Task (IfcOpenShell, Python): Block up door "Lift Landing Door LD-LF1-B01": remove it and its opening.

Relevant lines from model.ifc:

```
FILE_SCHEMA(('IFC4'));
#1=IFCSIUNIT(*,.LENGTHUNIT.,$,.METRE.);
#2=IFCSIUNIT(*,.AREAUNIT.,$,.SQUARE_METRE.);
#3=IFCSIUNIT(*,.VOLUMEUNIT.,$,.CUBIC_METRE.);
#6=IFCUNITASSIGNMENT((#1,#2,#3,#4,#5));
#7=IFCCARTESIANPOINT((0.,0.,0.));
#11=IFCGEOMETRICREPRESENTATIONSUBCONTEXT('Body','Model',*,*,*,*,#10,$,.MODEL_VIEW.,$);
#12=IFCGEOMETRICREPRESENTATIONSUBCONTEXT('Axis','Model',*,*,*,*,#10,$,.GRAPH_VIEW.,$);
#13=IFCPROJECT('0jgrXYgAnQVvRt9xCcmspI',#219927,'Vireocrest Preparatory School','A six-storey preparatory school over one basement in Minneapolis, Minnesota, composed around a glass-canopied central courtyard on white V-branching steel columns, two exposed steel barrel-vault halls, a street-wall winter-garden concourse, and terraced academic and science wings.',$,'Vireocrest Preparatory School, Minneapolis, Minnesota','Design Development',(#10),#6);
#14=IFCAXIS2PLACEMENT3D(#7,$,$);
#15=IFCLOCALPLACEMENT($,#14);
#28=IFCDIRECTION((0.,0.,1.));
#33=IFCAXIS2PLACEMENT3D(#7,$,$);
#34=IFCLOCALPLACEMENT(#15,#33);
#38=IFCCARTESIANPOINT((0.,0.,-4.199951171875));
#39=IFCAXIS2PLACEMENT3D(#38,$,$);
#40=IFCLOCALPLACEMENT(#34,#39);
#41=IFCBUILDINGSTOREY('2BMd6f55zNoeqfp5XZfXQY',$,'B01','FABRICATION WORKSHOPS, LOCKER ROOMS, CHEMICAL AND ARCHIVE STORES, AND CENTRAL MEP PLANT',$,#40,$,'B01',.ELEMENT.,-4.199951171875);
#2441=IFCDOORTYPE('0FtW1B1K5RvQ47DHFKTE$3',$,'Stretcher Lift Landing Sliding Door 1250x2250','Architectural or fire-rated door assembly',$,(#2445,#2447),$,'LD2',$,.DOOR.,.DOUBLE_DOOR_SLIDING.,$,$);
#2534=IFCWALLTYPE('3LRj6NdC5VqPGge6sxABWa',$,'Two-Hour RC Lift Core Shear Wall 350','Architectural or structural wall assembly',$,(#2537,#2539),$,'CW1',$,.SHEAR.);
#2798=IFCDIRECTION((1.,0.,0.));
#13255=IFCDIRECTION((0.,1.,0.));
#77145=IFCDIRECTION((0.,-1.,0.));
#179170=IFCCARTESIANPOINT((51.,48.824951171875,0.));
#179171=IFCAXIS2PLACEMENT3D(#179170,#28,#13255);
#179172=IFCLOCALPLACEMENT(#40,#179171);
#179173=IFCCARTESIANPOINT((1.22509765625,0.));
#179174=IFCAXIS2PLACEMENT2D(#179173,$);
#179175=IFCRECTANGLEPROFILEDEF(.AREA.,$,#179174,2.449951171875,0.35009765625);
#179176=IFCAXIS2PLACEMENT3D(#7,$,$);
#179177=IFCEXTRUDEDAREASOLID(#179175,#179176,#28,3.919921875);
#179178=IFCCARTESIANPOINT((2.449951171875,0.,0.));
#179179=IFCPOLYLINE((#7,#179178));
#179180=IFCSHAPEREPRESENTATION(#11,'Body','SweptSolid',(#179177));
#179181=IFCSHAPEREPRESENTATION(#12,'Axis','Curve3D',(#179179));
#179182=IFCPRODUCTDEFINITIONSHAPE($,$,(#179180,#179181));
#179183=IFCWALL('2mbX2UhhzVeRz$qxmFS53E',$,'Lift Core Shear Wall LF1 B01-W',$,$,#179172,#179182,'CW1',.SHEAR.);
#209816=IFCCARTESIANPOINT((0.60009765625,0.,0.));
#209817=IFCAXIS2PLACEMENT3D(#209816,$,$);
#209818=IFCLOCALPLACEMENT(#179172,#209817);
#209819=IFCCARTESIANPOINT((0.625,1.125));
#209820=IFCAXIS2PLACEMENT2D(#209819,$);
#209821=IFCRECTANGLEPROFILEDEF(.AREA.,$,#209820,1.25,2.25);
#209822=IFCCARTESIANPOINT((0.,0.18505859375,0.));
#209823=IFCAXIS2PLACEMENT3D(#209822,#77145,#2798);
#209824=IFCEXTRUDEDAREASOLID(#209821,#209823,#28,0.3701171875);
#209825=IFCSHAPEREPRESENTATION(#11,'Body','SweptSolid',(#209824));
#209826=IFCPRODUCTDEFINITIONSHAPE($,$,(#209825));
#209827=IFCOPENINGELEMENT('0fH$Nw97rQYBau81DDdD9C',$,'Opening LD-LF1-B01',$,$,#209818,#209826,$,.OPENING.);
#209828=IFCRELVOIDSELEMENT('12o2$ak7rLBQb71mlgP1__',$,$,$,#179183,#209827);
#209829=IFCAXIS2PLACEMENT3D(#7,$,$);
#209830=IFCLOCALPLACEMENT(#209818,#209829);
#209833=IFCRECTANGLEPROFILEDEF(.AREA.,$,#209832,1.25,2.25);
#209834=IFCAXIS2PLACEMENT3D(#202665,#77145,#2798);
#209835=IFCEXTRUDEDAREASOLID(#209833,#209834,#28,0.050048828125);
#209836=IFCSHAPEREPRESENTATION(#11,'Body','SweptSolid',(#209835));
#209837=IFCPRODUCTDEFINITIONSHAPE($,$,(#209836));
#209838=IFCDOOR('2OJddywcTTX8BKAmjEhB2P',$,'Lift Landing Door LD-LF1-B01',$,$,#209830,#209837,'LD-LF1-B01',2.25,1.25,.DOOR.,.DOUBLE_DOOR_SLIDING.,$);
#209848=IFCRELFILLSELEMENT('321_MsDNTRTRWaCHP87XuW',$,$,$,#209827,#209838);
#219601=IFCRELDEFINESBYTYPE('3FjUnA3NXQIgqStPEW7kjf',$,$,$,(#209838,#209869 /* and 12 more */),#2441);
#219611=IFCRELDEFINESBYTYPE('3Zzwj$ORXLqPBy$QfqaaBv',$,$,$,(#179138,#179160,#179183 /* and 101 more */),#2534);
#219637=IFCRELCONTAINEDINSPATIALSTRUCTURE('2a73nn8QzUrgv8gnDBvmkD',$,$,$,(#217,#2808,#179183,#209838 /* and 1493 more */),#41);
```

```python
import ifcopenshell
import ifcopenshell.api.feature
import ifcopenshell.api.root
import ifcopenshell.geom
import ifcopenshell.util.shape

model = ifcopenshell.open("model.ifc")
settings = ifcopenshell.geom.settings()


def volume(element):
    """Net volume in cubic metres, openings subtracted."""
    shape = ifcopenshell.geom.create_shape(settings, element)
    return ifcopenshell.util.shape.get_volume(shape.geometry)


door = model.by_guid("2OJddywcTTX8BKAmjEhB2P")
opening = door.FillsVoids[0].RelatingOpeningElement
wall = opening.VoidsElements[0].RelatingBuildingElement
before = volume(wall)

ifcopenshell.api.root.remove_product(model, product=door)
ifcopenshell.api.feature.remove_feature(model, feature=opening)

after = volume(wall)

print(f"wall volume {before:.3f} -> {after:.3f} m3")

model.write("model_v2.ifc")
```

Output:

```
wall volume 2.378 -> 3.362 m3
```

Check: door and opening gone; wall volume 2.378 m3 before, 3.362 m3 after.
